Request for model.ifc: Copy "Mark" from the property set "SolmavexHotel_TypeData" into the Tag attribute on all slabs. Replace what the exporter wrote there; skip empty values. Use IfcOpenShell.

First a look at what the model holds.

```python
import ifcopenshell
import ifcopenshell.util.element

model = ifcopenshell.open("model.ifc")
print(model.schema)
slabs = model.by_type("IfcSlab")
print(len(slabs), "slabs")
for e in slabs[:8]:
    source = ifcopenshell.util.element.get_pset(e, "SolmavexHotel_TypeData", "Mark")
    target = e.Tag
    print(e.id(), repr(source), repr(target), sep=" | ")
```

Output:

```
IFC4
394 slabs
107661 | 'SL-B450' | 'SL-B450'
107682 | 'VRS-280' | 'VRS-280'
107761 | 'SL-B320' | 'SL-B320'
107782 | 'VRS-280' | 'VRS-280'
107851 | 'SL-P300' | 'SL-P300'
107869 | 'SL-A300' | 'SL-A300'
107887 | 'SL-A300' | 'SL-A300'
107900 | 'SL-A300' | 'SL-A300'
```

```python
import ifcopenshell
import ifcopenshell.util.element

model = ifcopenshell.open("model.ifc")

count = 0
for e in model.by_type("IfcSlab"):
    value = ifcopenshell.util.element.get_pset(e, "SolmavexHotel_TypeData", "Mark")
    current = e.Tag
    if not value or not value.strip() or current == value:
        continue
    e.Tag = value
    count += 1

print(count, "slabs updated")

model.write("model_edited.ifc")
```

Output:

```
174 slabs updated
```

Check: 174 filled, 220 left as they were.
